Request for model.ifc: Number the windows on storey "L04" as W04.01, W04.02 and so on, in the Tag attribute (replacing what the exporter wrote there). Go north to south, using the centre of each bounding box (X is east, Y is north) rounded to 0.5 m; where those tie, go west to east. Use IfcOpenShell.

First a look at what the model holds.

```python
import ifcopenshell
import ifcopenshell.util.element
import ifcopenshell.util.placement

model = ifcopenshell.open("model.ifc")
print(model.schema)
storey = next(s for s in model.by_type("IfcBuildingStorey") if s.Name == "L04")
windows = [e for e in ifcopenshell.util.element.get_decomposition(storey) if e.is_a("IfcWindow")]
for e in sorted(windows, key=lambda e: e.id()):
    origin = ifcopenshell.util.placement.get_local_placement(e.ObjectPlacement)[:3, 3]
    print(e.id(), e.Tag, e.Name, origin.round(2) + 0.0, sep=" | ")
```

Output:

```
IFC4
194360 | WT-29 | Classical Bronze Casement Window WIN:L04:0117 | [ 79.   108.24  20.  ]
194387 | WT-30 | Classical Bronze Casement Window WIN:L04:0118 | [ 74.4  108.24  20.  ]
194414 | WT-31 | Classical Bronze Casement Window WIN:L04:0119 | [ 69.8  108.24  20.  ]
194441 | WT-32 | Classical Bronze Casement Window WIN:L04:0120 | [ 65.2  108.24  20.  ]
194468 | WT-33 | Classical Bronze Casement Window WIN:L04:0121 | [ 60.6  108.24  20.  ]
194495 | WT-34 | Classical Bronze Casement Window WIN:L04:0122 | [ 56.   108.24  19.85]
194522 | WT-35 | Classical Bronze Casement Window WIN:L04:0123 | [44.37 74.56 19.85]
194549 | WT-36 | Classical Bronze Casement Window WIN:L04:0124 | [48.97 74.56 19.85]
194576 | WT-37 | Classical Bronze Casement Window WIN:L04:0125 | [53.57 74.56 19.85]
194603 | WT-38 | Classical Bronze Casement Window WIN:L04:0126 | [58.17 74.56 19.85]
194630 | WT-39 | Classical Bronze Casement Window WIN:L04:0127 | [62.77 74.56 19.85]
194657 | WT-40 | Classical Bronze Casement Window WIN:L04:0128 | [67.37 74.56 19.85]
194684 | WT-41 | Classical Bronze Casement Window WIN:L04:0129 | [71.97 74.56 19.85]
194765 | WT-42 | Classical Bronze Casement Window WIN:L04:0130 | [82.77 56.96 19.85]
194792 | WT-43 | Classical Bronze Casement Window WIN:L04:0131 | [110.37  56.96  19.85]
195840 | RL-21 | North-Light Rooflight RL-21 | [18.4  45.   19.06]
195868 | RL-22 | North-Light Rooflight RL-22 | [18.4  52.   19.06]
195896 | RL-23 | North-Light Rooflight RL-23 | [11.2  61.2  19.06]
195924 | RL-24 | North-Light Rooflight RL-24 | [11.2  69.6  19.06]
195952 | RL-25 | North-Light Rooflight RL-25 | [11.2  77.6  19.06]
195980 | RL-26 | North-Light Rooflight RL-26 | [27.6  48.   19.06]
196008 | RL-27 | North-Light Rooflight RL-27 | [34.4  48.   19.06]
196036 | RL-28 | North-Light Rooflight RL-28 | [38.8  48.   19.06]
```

```python
import ifcopenshell
import ifcopenshell.geom
import ifcopenshell.util.element
import ifcopenshell.util.shape

model = ifcopenshell.open("model.ifc")
settings = ifcopenshell.geom.settings()
settings.set("use-world-coords", True)


def centre(element):
    shape = ifcopenshell.geom.create_shape(settings, element)
    return ifcopenshell.util.shape.get_bbox_centroid(shape.geometry)


storey = next(s for s in model.by_type("IfcBuildingStorey") if s.Name == "L04")
windows = [e for e in ifcopenshell.util.element.get_decomposition(storey) if e.is_a("IfcWindow")]

# Insertion points can sit at a corner or the storey origin, so sort by the geometry (in metres).
centres = {e: centre(e) for e in windows}
windows.sort(key=lambda e: (-round(centres[e][1] / 0.5), centres[e][0]))

for i, e in enumerate(windows, start=1):
    number = f"W04.{i:02d}"
    e.Tag = number
    print(e.id(), number)

model.write("model_v2.ifc")
```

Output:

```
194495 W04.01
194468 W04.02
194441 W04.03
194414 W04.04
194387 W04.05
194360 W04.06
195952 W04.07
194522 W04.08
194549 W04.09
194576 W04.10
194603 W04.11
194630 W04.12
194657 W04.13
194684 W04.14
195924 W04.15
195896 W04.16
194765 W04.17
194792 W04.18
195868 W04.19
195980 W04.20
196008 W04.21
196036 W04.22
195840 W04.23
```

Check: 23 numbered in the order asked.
